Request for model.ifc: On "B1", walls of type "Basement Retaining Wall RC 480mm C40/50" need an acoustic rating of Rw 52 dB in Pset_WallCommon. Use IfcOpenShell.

First a look at what the model holds.

```python
import ifcopenshell
import ifcopenshell.util.element

model = ifcopenshell.open("model.ifc")
print(model.schema)
storey = next(s for s in model.by_type("IfcBuildingStorey") if s.Name == "B1")
walls = [e for e in ifcopenshell.util.element.get_decomposition(storey) if e.is_a("IfcWall")]
seen = {}
for e in walls:
    element_type = ifcopenshell.util.element.get_type(e)
    key = (element_type.Name if element_type != e and element_type else None, ifcopenshell.util.element.get_pset(e, "Pset_WallCommon", "AcousticRating"))
    seen[key] = seen.get(key, 0) + 1
for (name, value), count in sorted(seen.items(), key=str):
    print(count, "x", name, "|", value)
```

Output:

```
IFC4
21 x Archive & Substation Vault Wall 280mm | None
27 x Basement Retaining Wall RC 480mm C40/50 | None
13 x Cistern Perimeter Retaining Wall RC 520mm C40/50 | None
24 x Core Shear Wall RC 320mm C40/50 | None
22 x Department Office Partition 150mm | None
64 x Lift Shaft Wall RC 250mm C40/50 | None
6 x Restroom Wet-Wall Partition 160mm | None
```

```python
import ifcopenshell
import ifcopenshell.api.pset
import ifcopenshell.util.element

model = ifcopenshell.open("model.ifc")

storey = next(s for s in model.by_type("IfcBuildingStorey") if s.Name == "B1")
walls = [e for e in ifcopenshell.util.element.get_decomposition(storey) if e.is_a("IfcWall")]

count = 0
for e in walls:
    element_type = ifcopenshell.util.element.get_type(e)
    if element_type in (None, e) or element_type.Name != "Basement Retaining Wall RC 480mm C40/50":
        continue
    # add_pset returns the element's existing set when there is one.
    pset = ifcopenshell.api.pset.add_pset(model, product=e, name="Pset_WallCommon")
    ifcopenshell.api.pset.edit_pset(model, pset=pset, properties={"AcousticRating": "Rw 52 dB"})
    count += 1

print(count, "walls updated")

model.write("model_rev.ifc")
```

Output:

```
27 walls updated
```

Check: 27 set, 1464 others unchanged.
